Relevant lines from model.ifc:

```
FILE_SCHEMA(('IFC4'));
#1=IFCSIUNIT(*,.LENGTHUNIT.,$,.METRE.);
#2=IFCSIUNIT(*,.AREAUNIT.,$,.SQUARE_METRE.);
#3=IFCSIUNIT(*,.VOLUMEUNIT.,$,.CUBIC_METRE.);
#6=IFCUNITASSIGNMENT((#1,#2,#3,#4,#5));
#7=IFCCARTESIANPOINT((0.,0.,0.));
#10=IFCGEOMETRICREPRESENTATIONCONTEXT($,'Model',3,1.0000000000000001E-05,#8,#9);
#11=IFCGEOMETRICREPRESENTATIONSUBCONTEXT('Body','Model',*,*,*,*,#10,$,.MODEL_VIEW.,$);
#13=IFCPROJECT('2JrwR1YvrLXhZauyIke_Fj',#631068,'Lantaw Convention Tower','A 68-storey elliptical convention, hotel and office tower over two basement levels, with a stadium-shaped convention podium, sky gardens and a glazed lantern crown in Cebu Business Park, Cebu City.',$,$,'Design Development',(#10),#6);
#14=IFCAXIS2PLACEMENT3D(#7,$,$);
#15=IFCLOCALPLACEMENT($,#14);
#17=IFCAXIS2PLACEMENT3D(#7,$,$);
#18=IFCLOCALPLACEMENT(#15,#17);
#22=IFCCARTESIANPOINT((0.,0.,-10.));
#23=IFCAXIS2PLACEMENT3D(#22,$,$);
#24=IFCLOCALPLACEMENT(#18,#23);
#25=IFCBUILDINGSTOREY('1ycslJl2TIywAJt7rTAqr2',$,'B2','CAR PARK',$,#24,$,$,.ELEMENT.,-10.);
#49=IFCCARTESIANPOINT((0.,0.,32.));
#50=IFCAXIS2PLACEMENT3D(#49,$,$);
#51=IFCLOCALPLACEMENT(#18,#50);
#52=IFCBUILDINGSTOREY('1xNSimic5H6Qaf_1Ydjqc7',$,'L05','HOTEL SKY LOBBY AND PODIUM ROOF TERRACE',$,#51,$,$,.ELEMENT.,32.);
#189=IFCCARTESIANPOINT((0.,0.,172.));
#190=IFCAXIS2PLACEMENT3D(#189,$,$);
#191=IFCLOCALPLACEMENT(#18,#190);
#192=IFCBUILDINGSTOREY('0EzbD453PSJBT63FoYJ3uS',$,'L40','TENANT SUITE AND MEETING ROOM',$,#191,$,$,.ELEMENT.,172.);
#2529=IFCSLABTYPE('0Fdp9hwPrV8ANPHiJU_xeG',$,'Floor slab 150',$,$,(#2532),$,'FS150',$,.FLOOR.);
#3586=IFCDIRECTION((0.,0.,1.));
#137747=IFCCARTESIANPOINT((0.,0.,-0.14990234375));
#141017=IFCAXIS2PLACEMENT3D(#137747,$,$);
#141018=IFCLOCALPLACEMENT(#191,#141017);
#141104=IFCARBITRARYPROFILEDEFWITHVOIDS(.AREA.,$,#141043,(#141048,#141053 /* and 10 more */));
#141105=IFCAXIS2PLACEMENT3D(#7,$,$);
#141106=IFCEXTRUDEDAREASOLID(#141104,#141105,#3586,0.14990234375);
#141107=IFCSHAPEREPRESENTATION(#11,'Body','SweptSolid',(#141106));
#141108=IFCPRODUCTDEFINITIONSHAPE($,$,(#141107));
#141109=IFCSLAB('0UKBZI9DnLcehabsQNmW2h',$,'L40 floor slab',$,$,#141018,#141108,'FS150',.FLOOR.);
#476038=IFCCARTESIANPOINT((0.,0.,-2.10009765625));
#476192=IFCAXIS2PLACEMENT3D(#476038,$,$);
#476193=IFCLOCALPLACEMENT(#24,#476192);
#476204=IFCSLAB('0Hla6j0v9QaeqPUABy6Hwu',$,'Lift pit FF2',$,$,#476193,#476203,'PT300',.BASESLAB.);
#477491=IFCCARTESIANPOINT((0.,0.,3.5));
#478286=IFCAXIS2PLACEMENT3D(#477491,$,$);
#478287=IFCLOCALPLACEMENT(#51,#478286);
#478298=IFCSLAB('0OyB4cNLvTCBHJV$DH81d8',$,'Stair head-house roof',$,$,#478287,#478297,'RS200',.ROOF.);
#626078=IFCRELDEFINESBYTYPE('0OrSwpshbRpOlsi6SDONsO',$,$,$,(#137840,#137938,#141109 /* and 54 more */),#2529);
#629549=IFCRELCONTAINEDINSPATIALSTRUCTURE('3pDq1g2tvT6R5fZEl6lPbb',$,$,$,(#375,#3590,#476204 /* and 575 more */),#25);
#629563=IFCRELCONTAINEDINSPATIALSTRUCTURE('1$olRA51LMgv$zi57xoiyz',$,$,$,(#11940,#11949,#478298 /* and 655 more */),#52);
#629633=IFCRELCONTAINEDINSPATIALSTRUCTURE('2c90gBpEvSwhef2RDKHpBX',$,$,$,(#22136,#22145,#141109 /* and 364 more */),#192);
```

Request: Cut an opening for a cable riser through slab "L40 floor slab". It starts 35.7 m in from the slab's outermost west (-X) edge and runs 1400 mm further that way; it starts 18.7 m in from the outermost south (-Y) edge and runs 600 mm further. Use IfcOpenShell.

```python
import numpy as np
import ifcopenshell
import ifcopenshell.api.feature
import ifcopenshell.api.geometry
import ifcopenshell.api.root
import ifcopenshell.geom
import ifcopenshell.util.placement
import ifcopenshell.util.representation
import ifcopenshell.util.shape
import ifcopenshell.util.unit

model = ifcopenshell.open("model.ifc")
unit_scale = ifcopenshell.util.unit.calculate_unit_scale(model)
settings = ifcopenshell.geom.settings()


def volume(element):
    """Net volume in cubic metres, openings subtracted."""
    shape = ifcopenshell.geom.create_shape(settings, element)
    return ifcopenshell.util.shape.get_volume(shape.geometry)


slab = model.by_guid("0UKBZI9DnLcehabsQNmW2h")
before = volume(slab)

# Extent in the slab's own axes, in metres. The edges named are its -X and -Y sides.
slab_shape = ifcopenshell.geom.create_shape(settings, slab)
vertices = ifcopenshell.util.shape.get_vertices(slab_shape.geometry)
x_min, y_min, bottom = vertices.min(axis=0)
top = vertices[:, 2].max()

opening = ifcopenshell.api.root.create_entity(model, ifc_class="IfcOpeningElement", name="Cable riser opening", predefined_type="OPENING")
context = ifcopenshell.util.representation.get_context(model, "Model", "Body", "MODEL_VIEW")
width, depth = 1.4, 0.6
outline = [(0.0, 0.0), (width, 0.0), (width, depth), (0.0, depth), (0.0, 0.0)]
# Overshoot both faces by 50 mm so the cut is clean.
shape = ifcopenshell.api.geometry.add_slab_representation(
    model, context=context, depth=top - bottom + 0.1, polyline=outline
)
ifcopenshell.api.geometry.assign_representation(model, product=opening, representation=shape)

matrix = ifcopenshell.util.placement.get_local_placement(slab.ObjectPlacement)
matrix[:, 3] = matrix @ np.append(np.array([x_min + 35.7, y_min + 18.7, bottom - 0.05]) / unit_scale, 1.0)
ifcopenshell.api.geometry.edit_object_placement(model, product=opening, matrix=matrix, is_si=False)
ifcopenshell.api.feature.add_feature(model, feature=opening, element=slab)

after = volume(slab)

print(f"slab volume {before:.3f} -> {after:.3f} m3")

model.write("model_edited.ifc")
```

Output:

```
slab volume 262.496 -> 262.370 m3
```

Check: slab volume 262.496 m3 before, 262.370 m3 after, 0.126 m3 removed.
